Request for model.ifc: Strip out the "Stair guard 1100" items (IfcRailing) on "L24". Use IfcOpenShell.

First a look at what the model holds.

```python
import ifcopenshell
import ifcopenshell.util.element

model = ifcopenshell.open("model.ifc")
print(model.schema)
storey = next(s for s in model.by_type("IfcBuildingStorey") if s.Name == "L24")
railings = [e for e in ifcopenshell.util.element.get_decomposition(storey) if e.is_a("IfcRailing")]
seen = {}
for e in railings:
    element_type = ifcopenshell.util.element.get_type(e)
    name = element_type.Name if element_type not in (None, e) else None
    seen[name] = seen.get(name, 0) + 1
for name, count in sorted(seen.items(), key=str):
    print(count, "x", name)
```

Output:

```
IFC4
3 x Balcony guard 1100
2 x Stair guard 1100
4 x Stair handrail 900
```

```python
import ifcopenshell
import ifcopenshell.api.root
import ifcopenshell.util.element

model = ifcopenshell.open("model.ifc")

storey = next(s for s in model.by_type("IfcBuildingStorey") if s.Name == "L24")
railings = [e for e in ifcopenshell.util.element.get_decomposition(storey) if e.is_a("IfcRailing")]
targets = [e for e in railings if (t := ifcopenshell.util.element.get_type(e)) not in (None, e) and t.Name == "Stair guard 1100"]

for e in targets:
    ifcopenshell.api.root.remove_product(model, product=e)
print(len(targets), "removed")

model.write("model_updated.ifc")
```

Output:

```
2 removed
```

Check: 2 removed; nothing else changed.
